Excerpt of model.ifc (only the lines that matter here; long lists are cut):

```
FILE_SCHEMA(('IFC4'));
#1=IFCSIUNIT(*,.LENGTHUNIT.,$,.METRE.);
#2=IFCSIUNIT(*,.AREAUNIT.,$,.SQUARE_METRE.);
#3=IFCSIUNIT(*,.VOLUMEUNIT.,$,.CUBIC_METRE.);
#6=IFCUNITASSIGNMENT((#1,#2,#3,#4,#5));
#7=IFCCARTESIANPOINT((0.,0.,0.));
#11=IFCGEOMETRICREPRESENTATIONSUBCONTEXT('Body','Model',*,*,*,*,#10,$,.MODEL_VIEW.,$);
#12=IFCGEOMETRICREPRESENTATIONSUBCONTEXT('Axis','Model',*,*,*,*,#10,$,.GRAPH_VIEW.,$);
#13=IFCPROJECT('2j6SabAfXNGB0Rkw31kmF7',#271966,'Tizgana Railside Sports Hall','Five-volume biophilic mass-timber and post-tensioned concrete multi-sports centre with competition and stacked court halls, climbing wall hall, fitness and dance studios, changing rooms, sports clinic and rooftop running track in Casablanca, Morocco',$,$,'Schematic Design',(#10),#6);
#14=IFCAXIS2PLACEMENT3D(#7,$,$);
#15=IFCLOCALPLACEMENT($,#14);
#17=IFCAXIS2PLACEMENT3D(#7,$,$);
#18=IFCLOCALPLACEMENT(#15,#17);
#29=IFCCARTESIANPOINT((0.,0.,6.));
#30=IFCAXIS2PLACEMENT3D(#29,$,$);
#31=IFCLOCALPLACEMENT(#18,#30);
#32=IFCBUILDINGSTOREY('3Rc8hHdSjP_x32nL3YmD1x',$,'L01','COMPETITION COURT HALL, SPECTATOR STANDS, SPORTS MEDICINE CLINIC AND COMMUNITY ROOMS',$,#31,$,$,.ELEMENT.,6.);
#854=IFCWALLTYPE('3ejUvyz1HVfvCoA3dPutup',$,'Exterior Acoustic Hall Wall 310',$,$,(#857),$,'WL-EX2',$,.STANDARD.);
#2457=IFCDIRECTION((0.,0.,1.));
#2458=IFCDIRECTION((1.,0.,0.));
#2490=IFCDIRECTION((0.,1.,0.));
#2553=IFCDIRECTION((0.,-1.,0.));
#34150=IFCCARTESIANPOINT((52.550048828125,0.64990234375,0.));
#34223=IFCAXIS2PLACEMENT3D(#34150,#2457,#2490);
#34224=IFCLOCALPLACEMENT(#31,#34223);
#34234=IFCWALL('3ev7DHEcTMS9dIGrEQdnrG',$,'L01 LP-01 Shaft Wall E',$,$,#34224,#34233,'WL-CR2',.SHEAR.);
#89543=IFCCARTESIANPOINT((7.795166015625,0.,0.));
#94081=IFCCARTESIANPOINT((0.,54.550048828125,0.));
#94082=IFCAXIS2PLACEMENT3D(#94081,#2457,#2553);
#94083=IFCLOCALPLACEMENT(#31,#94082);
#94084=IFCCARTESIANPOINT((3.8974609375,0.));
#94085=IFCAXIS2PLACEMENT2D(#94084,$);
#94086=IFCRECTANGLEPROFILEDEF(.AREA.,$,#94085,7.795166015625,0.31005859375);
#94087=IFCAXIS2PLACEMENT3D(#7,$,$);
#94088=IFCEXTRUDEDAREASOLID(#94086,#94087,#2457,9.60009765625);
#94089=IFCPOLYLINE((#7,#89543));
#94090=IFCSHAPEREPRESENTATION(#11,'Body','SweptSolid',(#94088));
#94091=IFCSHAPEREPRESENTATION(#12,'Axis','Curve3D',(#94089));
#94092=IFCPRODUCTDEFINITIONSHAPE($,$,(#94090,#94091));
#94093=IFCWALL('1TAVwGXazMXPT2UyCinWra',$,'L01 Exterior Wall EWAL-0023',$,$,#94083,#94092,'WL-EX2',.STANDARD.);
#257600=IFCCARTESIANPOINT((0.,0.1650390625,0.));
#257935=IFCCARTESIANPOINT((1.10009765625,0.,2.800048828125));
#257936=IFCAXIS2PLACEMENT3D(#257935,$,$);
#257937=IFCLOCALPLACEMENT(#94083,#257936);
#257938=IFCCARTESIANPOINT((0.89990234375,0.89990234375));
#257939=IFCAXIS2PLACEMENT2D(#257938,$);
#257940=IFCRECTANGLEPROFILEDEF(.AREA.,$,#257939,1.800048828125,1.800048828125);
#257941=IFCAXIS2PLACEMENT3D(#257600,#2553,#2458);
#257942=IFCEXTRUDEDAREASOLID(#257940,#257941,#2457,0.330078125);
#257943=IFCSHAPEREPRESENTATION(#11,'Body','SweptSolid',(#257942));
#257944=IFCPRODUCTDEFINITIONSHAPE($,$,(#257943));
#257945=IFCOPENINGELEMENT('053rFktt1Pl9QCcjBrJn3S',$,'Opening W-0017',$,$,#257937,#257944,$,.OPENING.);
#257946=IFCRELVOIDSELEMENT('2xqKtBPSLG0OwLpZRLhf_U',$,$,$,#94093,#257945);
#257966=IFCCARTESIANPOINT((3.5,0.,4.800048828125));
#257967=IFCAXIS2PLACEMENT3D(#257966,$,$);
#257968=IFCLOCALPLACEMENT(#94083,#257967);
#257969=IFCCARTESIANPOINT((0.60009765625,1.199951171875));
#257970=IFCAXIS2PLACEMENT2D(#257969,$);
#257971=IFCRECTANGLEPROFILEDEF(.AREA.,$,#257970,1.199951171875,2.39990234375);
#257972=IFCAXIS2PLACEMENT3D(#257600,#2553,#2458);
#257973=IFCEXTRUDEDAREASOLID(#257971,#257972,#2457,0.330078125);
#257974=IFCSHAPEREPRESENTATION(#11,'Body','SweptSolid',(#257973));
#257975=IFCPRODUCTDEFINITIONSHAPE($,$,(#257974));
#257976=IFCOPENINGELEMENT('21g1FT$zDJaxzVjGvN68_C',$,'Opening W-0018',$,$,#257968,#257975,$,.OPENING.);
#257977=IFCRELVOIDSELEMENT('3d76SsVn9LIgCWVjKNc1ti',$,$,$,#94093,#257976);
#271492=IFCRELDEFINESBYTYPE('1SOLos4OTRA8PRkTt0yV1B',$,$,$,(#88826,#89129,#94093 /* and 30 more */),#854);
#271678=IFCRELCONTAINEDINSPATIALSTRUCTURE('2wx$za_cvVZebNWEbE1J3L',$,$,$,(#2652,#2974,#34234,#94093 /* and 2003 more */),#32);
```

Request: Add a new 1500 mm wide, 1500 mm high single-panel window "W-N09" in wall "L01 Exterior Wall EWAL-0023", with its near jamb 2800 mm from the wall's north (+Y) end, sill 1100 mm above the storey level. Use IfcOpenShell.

```python
import numpy as np
import ifcopenshell
import ifcopenshell.api.feature
import ifcopenshell.api.geometry
import ifcopenshell.api.root
import ifcopenshell.api.spatial
import ifcopenshell.geom
import ifcopenshell.util.element
import ifcopenshell.util.placement
import ifcopenshell.util.representation
import ifcopenshell.util.shape
import ifcopenshell.util.unit

model = ifcopenshell.open("model.ifc")
unit_scale = ifcopenshell.util.unit.calculate_unit_scale(model)
settings = ifcopenshell.geom.settings()


def volume(element):
    """Net volume in cubic metres, openings subtracted."""
    shape = ifcopenshell.geom.create_shape(settings, element)
    return ifcopenshell.util.shape.get_volume(shape.geometry)


wall = model.by_guid("1TAVwGXazMXPT2UyCinWra")
storey = ifcopenshell.util.element.get_container(wall, ifc_class="IfcBuildingStorey")
context = ifcopenshell.util.representation.get_context(model, "Model", "Body", "MODEL_VIEW")
before = volume(wall)

width, height, from_end, sill = 1.5, 1.5, 2.8, 1.1  # metres

# The wall runs along its own X axis, and the end named is its -X end.
wall_shape = ifcopenshell.geom.create_shape(settings, wall)
x, y, z = ifcopenshell.util.shape.get_vertices(wall_shape.geometry).T
start = x.min() + from_end
face, thickness = float(y.min()), float(y.max() - y.min())
wall_matrix = ifcopenshell.util.placement.get_local_placement(wall.ObjectPlacement)
level = ifcopenshell.util.placement.get_local_placement(storey.ObjectPlacement)[2, 3]


def in_wall(x, y):
    """Placement at x, y metres in the wall's axes, at sill height."""
    matrix = wall_matrix.copy()
    matrix[:, 3] = wall_matrix @ np.array([x / unit_scale, y / unit_scale, 0.0, 1.0])
    matrix[2, 3] = level + sill / unit_scale
    return matrix


# Opening: a box that overshoots both wall faces by 50 mm.
opening = ifcopenshell.api.root.create_entity(model, ifc_class="IfcOpeningElement", predefined_type="OPENING")
box = ifcopenshell.api.geometry.add_wall_representation(
    model, context=context, length=width, height=height, thickness=thickness + 0.1
)
ifcopenshell.api.geometry.assign_representation(model, product=opening, representation=box)
ifcopenshell.api.geometry.edit_object_placement(model, product=opening, matrix=in_wall(start, face - 0.05), is_si=False)
ifcopenshell.api.feature.add_feature(model, feature=opening, element=wall)

window = ifcopenshell.api.root.create_entity(model, ifc_class="IfcWindow", name="W-N09", predefined_type="WINDOW")
window.OverallWidth, window.OverallHeight = width / unit_scale, height / unit_scale
window.PartitioningType = "SINGLE_PANEL"
body = ifcopenshell.api.geometry.add_window_representation(
    model,
    context=context,
    overall_width=window.OverallWidth,
    overall_height=window.OverallHeight,
    partition_type="SINGLE_PANEL",
)
ifcopenshell.api.geometry.assign_representation(model, product=window, representation=body)
ifcopenshell.api.spatial.assign_container(model, products=[window], relating_structure=storey)
ifcopenshell.api.feature.add_filling(model, opening=opening, element=window)

# Centre the window in the wall's thickness.
ifcopenshell.api.geometry.edit_object_placement(model, product=window, matrix=in_wall(start, face), is_si=False)
window_shape = ifcopenshell.geom.create_shape(settings, window)
depth = ifcopenshell.util.shape.get_vertices(window_shape.geometry)[:, 1]
offset = face + thickness / 2 - (depth.min() + depth.max()) / 2
ifcopenshell.api.geometry.edit_object_placement(model, product=window, matrix=in_wall(start, offset), is_si=False)

after = volume(wall)

print(f"wall volume {before:.3f} -> {after:.3f} m3")

model.write("model_edited.ifc")
```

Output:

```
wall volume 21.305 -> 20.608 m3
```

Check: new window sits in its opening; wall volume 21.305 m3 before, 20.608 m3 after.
